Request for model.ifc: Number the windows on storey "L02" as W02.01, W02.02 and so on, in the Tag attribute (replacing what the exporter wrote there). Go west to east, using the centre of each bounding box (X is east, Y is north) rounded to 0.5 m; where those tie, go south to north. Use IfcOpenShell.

First a look at what the model holds.

```python
import ifcopenshell
import ifcopenshell.util.element
import ifcopenshell.util.placement

model = ifcopenshell.open("model.ifc")
print(model.schema)
storey = next(s for s in model.by_type("IfcBuildingStorey") if s.Name == "L02")
windows = [e for e in ifcopenshell.util.element.get_decomposition(storey) if e.is_a("IfcWindow")]
for e in sorted(windows, key=lambda e: e.id()):
    origin = ifcopenshell.util.placement.get_local_placement(e.ObjectPlacement)[:3, 3]
    print(e.id(), e.Tag, e.Name, origin.round(2) + 0.0, sep=" | ")
```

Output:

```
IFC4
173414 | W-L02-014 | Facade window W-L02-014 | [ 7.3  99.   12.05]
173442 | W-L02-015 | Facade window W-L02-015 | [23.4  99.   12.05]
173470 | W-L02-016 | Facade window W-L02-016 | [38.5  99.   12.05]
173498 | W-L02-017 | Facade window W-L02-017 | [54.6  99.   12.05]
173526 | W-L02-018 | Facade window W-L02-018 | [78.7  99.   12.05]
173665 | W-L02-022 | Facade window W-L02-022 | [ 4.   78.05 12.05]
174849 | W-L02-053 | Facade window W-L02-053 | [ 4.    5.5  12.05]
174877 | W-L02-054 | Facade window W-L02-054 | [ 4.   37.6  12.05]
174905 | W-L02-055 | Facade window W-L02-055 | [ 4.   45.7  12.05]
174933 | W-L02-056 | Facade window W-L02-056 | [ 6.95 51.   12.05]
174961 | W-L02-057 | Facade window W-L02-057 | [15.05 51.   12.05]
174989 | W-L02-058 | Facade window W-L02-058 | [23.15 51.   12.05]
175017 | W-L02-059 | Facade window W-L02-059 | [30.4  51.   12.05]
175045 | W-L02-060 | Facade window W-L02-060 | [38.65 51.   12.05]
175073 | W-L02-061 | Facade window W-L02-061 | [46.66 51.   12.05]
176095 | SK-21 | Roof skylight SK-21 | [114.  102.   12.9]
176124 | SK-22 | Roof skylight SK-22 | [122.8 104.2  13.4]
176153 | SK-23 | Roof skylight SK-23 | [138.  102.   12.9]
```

```python
import ifcopenshell
import ifcopenshell.geom
import ifcopenshell.util.element
import ifcopenshell.util.shape

model = ifcopenshell.open("model.ifc")
settings = ifcopenshell.geom.settings()
settings.set("use-world-coords", True)


def centre(element):
    shape = ifcopenshell.geom.create_shape(settings, element)
    return ifcopenshell.util.shape.get_bbox_centroid(shape.geometry)


storey = next(s for s in model.by_type("IfcBuildingStorey") if s.Name == "L02")
windows = [e for e in ifcopenshell.util.element.get_decomposition(storey) if e.is_a("IfcWindow")]

# Insertion points can sit at a corner or the storey origin, so sort by the geometry (in metres).
centres = {e: centre(e) for e in windows}
windows.sort(key=lambda e: (round(centres[e][0] / 0.5), centres[e][1]))

for i, e in enumerate(windows, start=1):
    number = f"W02.{i:02d}"
    e.Tag = number
    print(e.id(), number)

model.write("model-out.ifc")
```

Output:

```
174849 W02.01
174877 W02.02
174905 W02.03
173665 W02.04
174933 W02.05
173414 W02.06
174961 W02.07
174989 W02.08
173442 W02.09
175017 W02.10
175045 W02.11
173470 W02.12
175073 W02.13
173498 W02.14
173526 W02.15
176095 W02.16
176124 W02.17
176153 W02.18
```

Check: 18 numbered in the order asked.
